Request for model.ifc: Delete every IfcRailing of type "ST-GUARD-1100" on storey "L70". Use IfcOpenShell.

First a look at what the model holds.

```python
import ifcopenshell
import ifcopenshell.util.element

model = ifcopenshell.open("model.ifc")
print(model.schema)
storey = next(s for s in model.by_type("IfcBuildingStorey") if s.Name == "L70")
railings = [e for e in ifcopenshell.util.element.get_decomposition(storey) if e.is_a("IfcRailing")]
seen = {}
for e in railings:
    element_type = ifcopenshell.util.element.get_type(e)
    name = element_type.Name if element_type not in (None, e) else None
    seen[name] = seen.get(name, 0) + 1
for name, count in sorted(seen.items(), key=str):
    print(count, "x", name)
```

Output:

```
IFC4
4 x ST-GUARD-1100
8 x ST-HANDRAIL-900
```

```python
import ifcopenshell
import ifcopenshell.api.root
import ifcopenshell.util.element

model = ifcopenshell.open("model.ifc")

storey = next(s for s in model.by_type("IfcBuildingStorey") if s.Name == "L70")
railings = [e for e in ifcopenshell.util.element.get_decomposition(storey) if e.is_a("IfcRailing")]
targets = [e for e in railings if (t := ifcopenshell.util.element.get_type(e)) not in (None, e) and t.Name == "ST-GUARD-1100"]

for e in targets:
    ifcopenshell.api.root.remove_product(model, product=e)
print(len(targets), "removed")

model.write("model-out.ifc")
```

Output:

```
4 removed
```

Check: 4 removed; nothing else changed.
